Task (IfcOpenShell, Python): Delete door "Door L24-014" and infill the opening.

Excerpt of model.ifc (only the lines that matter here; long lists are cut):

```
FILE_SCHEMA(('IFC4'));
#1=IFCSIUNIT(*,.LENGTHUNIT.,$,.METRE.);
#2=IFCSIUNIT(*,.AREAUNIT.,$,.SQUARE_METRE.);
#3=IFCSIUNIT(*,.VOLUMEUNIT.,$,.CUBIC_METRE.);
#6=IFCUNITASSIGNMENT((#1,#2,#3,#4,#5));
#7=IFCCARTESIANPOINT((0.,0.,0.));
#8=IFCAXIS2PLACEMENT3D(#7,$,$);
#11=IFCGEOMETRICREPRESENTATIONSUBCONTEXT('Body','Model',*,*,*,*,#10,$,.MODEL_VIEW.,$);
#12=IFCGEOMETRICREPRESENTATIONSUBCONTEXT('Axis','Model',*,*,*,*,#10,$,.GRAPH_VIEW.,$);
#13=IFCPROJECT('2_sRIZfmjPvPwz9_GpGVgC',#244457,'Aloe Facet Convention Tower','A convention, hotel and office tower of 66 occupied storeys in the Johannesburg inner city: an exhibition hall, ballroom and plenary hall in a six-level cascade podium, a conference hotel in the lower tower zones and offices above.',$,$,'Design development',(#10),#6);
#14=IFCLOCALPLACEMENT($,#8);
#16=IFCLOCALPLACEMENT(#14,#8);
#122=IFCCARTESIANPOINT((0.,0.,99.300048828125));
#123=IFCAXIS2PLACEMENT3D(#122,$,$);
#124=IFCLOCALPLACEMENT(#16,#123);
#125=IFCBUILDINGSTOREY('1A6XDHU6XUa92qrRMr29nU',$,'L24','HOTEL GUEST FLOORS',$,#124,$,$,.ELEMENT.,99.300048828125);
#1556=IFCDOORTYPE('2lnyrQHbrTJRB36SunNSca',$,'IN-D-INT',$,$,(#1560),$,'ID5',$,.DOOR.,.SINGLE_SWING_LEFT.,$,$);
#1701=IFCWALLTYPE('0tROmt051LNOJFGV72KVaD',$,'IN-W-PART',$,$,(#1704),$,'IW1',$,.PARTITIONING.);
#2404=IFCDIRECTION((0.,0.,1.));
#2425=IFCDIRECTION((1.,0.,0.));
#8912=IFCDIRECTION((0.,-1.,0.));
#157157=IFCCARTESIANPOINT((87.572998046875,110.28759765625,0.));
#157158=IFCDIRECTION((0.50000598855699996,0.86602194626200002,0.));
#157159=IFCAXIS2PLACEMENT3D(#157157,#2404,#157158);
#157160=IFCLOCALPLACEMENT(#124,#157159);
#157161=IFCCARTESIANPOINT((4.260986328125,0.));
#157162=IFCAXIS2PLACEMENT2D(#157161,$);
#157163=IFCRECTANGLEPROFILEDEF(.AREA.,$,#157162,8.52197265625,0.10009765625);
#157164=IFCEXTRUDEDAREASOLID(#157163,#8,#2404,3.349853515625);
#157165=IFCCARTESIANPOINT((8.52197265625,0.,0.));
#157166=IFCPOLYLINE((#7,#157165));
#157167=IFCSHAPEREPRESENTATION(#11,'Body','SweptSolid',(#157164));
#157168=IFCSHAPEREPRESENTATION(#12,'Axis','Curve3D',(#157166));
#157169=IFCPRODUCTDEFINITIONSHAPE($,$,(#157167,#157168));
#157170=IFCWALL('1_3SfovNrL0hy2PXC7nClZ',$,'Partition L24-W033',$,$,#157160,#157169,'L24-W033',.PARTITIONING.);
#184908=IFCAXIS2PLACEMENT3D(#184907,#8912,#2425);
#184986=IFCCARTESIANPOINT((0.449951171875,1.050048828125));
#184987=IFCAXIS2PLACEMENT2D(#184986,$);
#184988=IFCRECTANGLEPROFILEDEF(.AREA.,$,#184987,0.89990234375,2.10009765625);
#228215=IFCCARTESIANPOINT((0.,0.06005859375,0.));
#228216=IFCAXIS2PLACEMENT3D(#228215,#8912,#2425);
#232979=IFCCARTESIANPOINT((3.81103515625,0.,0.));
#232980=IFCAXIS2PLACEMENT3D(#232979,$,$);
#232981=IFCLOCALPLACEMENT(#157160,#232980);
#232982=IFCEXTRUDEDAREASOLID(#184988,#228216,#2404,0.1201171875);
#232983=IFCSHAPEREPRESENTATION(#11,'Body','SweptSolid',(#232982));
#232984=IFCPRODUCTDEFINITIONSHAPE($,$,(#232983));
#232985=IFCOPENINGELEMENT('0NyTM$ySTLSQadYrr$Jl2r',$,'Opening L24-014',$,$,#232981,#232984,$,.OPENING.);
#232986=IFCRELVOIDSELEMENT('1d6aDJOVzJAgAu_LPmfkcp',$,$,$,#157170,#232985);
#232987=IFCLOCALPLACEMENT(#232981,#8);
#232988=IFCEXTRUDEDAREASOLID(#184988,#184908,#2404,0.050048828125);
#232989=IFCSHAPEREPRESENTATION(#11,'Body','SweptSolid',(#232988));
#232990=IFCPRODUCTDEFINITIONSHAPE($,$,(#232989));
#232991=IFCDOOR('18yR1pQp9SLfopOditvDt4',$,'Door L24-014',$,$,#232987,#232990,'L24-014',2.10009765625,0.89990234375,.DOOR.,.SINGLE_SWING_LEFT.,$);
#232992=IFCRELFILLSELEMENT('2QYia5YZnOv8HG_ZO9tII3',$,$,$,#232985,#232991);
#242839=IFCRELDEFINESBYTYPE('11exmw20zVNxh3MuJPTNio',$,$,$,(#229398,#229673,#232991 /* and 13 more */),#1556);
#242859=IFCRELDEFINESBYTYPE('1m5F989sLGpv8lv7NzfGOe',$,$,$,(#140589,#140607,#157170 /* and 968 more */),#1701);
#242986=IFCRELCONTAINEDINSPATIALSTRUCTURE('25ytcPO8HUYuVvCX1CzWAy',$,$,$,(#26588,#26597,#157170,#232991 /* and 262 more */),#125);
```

```python
import ifcopenshell
import ifcopenshell.api.feature
import ifcopenshell.api.root
import ifcopenshell.geom
import ifcopenshell.util.shape

model = ifcopenshell.open("model.ifc")
settings = ifcopenshell.geom.settings()


def volume(element):
    """Net volume in cubic metres, openings subtracted."""
    shape = ifcopenshell.geom.create_shape(settings, element)
    return ifcopenshell.util.shape.get_volume(shape.geometry)


door = model.by_guid("18yR1pQp9SLfopOditvDt4")
opening = door.FillsVoids[0].RelatingOpeningElement
wall = opening.VoidsElements[0].RelatingBuildingElement
before = volume(wall)

ifcopenshell.api.root.remove_product(model, product=door)
ifcopenshell.api.feature.remove_feature(model, feature=opening)

after = volume(wall)

print(f"wall volume {before:.3f} -> {after:.3f} m3")

model.write("model_updated.ifc")
```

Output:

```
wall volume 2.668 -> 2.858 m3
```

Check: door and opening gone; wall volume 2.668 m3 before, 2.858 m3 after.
